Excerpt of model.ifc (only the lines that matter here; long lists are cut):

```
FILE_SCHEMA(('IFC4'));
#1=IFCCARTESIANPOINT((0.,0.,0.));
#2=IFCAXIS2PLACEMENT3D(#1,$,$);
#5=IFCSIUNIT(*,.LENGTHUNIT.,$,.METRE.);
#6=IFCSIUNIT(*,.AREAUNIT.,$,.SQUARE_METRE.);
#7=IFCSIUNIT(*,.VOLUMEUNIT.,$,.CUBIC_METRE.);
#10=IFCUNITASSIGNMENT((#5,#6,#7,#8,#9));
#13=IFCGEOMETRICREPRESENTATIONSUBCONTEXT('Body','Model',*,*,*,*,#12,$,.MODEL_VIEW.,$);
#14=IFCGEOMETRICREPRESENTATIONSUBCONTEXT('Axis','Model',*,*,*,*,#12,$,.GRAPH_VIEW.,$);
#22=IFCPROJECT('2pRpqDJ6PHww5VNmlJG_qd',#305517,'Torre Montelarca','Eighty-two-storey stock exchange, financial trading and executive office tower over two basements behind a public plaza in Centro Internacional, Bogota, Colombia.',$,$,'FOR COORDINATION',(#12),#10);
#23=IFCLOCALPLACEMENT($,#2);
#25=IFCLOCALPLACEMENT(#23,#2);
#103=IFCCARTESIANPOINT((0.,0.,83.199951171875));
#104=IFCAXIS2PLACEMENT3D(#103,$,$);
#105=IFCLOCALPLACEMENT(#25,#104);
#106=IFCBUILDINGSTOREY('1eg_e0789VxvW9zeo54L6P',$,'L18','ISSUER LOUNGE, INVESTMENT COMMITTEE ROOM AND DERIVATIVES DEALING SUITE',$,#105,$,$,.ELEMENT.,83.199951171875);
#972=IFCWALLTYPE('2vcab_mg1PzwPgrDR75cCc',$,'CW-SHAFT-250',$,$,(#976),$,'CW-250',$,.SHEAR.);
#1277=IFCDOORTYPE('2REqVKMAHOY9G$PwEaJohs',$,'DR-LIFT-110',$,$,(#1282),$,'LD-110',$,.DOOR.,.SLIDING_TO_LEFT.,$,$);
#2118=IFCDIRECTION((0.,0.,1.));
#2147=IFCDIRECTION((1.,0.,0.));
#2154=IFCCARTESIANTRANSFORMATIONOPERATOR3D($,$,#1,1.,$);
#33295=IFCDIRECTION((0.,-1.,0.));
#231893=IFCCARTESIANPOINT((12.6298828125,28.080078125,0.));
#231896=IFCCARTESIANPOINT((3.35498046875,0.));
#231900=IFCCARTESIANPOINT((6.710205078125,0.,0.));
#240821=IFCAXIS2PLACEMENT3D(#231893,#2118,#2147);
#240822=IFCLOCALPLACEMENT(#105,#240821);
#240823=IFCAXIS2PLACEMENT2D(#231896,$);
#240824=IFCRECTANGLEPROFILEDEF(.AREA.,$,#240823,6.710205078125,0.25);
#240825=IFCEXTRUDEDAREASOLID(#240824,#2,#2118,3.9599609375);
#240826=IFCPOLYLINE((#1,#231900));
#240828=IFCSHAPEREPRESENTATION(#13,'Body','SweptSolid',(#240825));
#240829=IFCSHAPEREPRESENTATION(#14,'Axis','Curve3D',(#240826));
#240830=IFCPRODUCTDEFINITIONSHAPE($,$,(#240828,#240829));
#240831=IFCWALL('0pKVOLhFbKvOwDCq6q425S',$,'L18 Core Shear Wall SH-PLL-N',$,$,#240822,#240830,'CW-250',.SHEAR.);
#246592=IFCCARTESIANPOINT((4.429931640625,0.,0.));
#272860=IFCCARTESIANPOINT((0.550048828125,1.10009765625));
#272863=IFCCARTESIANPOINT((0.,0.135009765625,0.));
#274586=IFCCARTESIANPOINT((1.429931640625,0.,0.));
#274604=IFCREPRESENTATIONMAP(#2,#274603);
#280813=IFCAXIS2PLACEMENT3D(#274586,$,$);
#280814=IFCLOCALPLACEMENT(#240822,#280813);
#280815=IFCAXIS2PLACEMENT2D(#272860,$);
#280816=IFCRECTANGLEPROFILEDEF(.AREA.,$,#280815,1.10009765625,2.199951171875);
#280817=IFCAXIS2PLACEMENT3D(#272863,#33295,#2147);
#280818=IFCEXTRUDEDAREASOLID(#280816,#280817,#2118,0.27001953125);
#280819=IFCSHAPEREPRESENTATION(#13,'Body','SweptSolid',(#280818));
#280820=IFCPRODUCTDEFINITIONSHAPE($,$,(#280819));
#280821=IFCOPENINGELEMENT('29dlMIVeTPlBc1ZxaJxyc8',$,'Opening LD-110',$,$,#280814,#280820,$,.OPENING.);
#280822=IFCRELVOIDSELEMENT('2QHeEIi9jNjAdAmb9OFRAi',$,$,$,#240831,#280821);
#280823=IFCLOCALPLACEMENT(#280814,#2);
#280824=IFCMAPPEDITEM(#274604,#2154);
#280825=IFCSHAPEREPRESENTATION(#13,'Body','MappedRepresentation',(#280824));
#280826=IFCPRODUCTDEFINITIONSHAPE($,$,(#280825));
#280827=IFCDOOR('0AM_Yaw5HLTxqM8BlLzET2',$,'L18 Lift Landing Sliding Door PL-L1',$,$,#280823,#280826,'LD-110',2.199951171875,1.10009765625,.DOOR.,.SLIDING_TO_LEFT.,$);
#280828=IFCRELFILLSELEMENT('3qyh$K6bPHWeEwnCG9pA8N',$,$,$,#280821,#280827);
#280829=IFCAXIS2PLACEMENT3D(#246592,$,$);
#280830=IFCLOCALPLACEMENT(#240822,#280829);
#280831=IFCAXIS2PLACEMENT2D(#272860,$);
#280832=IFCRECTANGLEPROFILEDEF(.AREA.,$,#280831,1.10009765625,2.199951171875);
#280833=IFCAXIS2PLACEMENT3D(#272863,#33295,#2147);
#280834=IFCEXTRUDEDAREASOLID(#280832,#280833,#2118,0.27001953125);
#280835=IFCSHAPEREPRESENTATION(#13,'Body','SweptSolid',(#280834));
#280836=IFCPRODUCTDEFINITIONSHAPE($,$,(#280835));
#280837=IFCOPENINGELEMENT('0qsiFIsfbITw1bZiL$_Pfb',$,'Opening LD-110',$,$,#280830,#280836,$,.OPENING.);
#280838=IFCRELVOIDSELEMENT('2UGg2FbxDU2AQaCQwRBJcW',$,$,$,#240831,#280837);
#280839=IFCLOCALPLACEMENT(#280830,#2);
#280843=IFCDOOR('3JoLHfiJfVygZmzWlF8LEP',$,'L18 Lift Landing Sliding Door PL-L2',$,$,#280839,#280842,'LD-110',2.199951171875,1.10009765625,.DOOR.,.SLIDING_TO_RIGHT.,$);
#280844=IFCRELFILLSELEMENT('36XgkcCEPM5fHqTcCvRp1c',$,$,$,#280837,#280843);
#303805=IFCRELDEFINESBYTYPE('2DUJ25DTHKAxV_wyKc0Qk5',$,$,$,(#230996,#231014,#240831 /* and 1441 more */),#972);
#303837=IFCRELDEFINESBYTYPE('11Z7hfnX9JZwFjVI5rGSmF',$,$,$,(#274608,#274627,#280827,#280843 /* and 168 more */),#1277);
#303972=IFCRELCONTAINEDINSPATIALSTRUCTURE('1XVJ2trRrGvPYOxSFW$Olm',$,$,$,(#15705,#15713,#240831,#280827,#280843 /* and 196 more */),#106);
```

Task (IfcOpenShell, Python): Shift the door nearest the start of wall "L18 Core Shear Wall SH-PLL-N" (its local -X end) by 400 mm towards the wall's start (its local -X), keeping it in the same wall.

```python
import ifcopenshell
import ifcopenshell.api.geometry
import ifcopenshell.util.placement
import ifcopenshell.util.unit

model = ifcopenshell.open("model.ifc")
unit_scale = ifcopenshell.util.unit.calculate_unit_scale(model)

door = model.by_guid("0AM_Yaw5HLTxqM8BlLzET2")
opening = door.FillsVoids[0].RelatingOpeningElement
wall = opening.VoidsElements[0].RelatingBuildingElement

wall_matrix = ifcopenshell.util.placement.get_local_placement(wall.ObjectPlacement)
shift = wall_matrix[:3, 0] * -0.4 / unit_scale
before = ifcopenshell.util.placement.get_local_placement(door.ObjectPlacement)[:3, 3].copy()

# The door is placed relative to its opening, so it follows when the opening moves.
matrix = ifcopenshell.util.placement.get_local_placement(opening.ObjectPlacement)
matrix[:3, 3] += shift
ifcopenshell.api.geometry.edit_object_placement(
    model, product=opening, matrix=matrix, is_si=False, should_transform_children=True
)

after = ifcopenshell.util.placement.get_local_placement(door.ObjectPlacement)[:3, 3]
print("door moved by", (after - before).round(3) + 0.0)

model.write("model-out.ifc")
```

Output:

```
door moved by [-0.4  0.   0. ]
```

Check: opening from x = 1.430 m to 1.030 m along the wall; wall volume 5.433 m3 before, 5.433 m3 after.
